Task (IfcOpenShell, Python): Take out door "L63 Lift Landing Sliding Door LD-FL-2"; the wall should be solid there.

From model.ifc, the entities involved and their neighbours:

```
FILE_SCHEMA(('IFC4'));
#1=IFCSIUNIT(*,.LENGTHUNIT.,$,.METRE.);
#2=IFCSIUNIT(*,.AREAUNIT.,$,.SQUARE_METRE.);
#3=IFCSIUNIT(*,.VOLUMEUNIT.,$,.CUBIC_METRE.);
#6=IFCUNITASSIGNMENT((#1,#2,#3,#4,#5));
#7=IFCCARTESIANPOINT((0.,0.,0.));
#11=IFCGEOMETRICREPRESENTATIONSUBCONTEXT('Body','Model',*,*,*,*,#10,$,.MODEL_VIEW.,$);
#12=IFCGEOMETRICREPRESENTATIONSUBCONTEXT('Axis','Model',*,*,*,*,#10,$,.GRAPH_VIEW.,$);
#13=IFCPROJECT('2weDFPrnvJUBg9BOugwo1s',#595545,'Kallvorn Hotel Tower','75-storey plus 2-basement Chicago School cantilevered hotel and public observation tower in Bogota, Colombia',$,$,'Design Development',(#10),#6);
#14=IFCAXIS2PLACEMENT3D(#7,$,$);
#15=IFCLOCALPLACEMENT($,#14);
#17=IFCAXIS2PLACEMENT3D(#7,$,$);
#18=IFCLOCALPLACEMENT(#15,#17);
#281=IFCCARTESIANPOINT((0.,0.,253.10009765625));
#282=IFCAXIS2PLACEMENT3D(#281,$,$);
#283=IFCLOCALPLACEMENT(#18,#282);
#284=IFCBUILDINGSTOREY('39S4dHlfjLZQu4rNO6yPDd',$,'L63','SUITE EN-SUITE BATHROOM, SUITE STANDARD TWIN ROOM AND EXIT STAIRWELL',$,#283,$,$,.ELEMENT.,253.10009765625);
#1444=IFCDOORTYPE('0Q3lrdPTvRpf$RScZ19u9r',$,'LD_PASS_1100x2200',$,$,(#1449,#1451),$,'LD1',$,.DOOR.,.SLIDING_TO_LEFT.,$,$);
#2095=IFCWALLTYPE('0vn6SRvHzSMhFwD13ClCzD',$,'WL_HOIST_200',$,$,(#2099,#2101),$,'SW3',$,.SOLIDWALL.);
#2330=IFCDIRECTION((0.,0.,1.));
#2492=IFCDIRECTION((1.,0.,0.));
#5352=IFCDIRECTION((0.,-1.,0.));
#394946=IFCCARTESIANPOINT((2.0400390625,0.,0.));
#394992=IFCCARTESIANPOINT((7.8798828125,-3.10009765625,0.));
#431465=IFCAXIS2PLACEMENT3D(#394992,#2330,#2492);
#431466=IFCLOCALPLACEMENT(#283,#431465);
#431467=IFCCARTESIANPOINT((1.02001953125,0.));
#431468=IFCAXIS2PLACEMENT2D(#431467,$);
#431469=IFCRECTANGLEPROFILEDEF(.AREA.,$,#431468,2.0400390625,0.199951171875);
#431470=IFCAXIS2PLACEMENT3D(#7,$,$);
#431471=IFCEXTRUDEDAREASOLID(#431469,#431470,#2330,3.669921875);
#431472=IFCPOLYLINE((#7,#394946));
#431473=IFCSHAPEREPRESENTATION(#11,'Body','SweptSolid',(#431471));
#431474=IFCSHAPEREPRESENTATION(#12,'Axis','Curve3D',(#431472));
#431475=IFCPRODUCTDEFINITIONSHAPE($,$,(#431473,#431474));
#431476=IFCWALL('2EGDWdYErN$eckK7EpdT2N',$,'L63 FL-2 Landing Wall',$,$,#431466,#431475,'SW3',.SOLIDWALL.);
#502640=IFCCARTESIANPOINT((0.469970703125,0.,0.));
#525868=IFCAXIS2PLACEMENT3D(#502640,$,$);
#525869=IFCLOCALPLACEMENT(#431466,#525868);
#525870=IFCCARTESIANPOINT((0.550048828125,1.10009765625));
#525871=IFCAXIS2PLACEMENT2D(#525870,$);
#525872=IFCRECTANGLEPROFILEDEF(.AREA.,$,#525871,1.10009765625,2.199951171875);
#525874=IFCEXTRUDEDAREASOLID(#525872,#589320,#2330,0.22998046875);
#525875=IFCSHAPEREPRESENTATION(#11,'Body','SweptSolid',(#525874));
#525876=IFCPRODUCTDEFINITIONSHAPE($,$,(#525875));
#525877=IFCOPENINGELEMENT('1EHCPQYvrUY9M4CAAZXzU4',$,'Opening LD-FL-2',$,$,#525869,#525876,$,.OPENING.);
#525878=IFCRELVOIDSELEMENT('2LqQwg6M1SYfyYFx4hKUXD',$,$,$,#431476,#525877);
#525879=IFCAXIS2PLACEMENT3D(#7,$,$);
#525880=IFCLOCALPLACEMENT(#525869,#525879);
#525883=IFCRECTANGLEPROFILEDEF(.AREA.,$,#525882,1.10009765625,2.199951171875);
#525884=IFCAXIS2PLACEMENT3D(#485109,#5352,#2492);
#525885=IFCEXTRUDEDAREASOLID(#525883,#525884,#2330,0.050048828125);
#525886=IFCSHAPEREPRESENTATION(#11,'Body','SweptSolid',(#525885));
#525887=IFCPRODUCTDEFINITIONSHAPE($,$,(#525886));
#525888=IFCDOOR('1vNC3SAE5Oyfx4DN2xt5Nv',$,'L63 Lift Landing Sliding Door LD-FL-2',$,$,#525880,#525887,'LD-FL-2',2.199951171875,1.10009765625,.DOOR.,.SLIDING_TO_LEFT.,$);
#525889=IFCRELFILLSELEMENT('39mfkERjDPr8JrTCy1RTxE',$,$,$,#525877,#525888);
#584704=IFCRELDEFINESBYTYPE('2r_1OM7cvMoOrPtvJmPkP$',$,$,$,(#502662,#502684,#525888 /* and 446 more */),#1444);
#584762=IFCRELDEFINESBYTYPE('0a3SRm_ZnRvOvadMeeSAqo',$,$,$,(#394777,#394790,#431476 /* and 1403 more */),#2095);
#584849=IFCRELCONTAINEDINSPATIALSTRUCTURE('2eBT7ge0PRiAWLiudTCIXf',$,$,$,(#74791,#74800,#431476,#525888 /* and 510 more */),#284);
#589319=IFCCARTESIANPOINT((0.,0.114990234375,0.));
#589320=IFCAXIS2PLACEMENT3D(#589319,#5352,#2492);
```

```python
import ifcopenshell
import ifcopenshell.api.feature
import ifcopenshell.api.root
import ifcopenshell.geom
import ifcopenshell.util.shape

model = ifcopenshell.open("model.ifc")
settings = ifcopenshell.geom.settings()


def volume(element):
    """Net volume in cubic metres, openings subtracted."""
    shape = ifcopenshell.geom.create_shape(settings, element)
    return ifcopenshell.util.shape.get_volume(shape.geometry)


door = model.by_id(525888)
opening = door.FillsVoids[0].RelatingOpeningElement
wall = opening.VoidsElements[0].RelatingBuildingElement
before = volume(wall)

ifcopenshell.api.root.remove_product(model, product=door)
ifcopenshell.api.feature.remove_feature(model, feature=opening)

after = volume(wall)

print(f"wall volume {before:.3f} -> {after:.3f} m3")

model.write("model_v2.ifc")
```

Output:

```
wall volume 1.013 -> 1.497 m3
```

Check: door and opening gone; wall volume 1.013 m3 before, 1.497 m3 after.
